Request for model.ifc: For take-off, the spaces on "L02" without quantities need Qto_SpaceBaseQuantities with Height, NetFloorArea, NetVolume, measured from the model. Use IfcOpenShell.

First a look at what the model holds.

```python
import ifcopenshell
import ifcopenshell.util.element
import ifcopenshell.util.unit

model = ifcopenshell.open("model.ifc")
print(model.schema)
for unit_type in ("LENGTHUNIT", "AREAUNIT", "VOLUMEUNIT"):
    print(unit_type, ifcopenshell.util.unit.calculate_unit_scale(model, unit_type))
storey = next(s for s in model.by_type("IfcBuildingStorey") if s.Name == "L02")
spaces = [e for e in ifcopenshell.util.element.get_decomposition(storey) if e.is_a("IfcSpace")]
for e in sorted(spaces, key=lambda e: e.id()):
    print(e.id(), e.is_a(), e.Name, list(ifcopenshell.util.element.get_psets(e, qtos_only=True)), sep=" | ")
```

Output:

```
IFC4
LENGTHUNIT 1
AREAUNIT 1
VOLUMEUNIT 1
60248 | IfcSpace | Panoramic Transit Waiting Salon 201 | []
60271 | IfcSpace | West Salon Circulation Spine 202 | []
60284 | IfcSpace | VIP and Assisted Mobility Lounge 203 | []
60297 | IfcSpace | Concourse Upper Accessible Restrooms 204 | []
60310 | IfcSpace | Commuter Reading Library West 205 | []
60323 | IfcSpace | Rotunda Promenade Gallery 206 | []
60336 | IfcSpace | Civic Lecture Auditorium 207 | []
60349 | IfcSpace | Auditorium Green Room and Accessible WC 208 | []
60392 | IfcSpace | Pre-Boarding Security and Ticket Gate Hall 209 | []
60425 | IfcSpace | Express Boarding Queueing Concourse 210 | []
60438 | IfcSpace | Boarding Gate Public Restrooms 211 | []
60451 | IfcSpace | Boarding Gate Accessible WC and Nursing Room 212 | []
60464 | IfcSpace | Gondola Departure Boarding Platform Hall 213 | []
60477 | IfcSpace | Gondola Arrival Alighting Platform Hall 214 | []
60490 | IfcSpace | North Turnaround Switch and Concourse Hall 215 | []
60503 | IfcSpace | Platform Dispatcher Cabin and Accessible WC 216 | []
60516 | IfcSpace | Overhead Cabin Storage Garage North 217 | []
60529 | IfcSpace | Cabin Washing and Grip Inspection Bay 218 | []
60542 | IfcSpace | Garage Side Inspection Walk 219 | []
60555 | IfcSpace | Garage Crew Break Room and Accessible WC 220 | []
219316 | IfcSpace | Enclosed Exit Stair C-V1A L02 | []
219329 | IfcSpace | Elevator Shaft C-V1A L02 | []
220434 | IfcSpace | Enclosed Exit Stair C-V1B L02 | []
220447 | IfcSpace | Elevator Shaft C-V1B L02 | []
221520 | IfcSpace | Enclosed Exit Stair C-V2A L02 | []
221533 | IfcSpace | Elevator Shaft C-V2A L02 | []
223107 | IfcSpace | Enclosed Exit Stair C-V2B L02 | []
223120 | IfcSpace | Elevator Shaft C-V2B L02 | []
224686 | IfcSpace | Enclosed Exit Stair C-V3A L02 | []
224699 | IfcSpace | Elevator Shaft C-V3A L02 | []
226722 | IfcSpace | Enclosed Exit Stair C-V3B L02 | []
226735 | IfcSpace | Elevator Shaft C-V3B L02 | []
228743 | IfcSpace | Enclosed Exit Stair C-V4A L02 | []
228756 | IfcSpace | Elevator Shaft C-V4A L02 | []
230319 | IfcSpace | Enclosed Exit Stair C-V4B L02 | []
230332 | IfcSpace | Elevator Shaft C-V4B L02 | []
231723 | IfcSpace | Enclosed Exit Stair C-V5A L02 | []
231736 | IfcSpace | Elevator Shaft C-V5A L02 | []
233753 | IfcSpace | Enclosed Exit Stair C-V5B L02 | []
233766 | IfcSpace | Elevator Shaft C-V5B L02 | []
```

```python
import ifcopenshell
import ifcopenshell.api.pset
import ifcopenshell.geom
import ifcopenshell.util.element
import ifcopenshell.util.shape
import ifcopenshell.util.unit

model = ifcopenshell.open("model.ifc")
unit_scale = ifcopenshell.util.unit.calculate_unit_scale(model)
area_scale = ifcopenshell.util.unit.calculate_unit_scale(model, "AREAUNIT")
volume_scale = ifcopenshell.util.unit.calculate_unit_scale(model, "VOLUMEUNIT")
settings = ifcopenshell.geom.settings()

storey = next(s for s in model.by_type("IfcBuildingStorey") if s.Name == "L02")
spaces = [e for e in ifcopenshell.util.element.get_decomposition(storey) if e.is_a("IfcSpace")]

for e in sorted(spaces, key=lambda e: e.id()):
    if ifcopenshell.util.element.get_psets(e, qtos_only=True, should_inherit=False):
        continue
    # Geometry comes back in metres, in the element's own axes.
    shape = ifcopenshell.geom.create_shape(settings, e)
    values = {
        "Height": ifcopenshell.util.shape.get_z(shape.geometry) / unit_scale,
        "NetFloorArea": ifcopenshell.util.shape.get_footprint_area(shape.geometry) / area_scale,
        "NetVolume": ifcopenshell.util.shape.get_volume(shape.geometry) / volume_scale,
    }
    qto = ifcopenshell.api.pset.add_qto(model, product=e, name="Qto_SpaceBaseQuantities")
    ifcopenshell.api.pset.edit_qto(model, qto=qto, properties=values)
    print(e.id(), {k: round(v, 3) for k, v in values.items()})

model.write("model_v2.ifc")
```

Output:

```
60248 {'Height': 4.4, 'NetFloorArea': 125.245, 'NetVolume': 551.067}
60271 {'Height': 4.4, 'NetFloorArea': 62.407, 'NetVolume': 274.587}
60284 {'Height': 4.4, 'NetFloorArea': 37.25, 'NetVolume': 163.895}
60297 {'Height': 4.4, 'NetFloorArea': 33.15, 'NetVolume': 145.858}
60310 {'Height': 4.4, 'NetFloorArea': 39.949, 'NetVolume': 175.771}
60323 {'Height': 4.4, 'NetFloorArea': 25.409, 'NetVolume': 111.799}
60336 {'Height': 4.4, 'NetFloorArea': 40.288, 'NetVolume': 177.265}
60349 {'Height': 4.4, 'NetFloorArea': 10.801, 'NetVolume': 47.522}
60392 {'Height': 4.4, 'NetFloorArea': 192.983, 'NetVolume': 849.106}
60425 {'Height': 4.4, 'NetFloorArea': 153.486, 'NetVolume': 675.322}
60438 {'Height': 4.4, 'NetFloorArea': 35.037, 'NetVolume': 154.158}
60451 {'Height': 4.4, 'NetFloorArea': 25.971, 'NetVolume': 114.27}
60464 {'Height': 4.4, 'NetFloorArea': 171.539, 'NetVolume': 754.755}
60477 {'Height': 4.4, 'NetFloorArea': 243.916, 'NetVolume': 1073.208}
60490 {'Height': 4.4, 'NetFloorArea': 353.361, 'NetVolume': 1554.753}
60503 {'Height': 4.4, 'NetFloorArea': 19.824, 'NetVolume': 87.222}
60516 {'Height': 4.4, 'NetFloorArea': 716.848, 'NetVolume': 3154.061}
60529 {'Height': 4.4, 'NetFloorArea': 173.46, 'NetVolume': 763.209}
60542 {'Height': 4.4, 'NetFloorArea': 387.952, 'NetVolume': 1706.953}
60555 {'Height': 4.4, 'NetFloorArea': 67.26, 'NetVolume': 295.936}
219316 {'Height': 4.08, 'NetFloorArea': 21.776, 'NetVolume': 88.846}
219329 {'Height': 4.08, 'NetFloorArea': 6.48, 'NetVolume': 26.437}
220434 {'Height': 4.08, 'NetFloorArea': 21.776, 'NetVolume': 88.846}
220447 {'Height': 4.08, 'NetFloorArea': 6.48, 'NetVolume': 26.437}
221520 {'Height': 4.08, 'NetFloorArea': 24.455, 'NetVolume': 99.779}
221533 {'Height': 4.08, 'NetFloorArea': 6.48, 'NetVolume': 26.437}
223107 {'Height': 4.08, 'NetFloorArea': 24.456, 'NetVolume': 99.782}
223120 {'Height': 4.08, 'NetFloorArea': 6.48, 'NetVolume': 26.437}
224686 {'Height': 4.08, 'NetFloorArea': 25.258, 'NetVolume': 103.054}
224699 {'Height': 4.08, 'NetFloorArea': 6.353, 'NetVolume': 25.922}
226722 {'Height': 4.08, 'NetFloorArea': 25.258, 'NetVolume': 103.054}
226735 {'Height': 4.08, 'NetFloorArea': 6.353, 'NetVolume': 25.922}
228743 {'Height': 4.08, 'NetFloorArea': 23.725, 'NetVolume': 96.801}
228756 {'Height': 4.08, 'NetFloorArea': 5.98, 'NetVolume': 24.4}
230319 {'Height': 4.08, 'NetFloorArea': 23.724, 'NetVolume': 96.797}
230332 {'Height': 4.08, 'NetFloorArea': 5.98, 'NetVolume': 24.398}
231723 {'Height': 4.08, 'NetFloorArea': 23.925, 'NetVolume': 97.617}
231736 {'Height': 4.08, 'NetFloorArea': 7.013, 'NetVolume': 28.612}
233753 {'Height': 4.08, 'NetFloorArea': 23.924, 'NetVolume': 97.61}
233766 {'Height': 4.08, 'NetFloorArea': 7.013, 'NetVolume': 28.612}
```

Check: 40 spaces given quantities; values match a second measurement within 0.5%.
